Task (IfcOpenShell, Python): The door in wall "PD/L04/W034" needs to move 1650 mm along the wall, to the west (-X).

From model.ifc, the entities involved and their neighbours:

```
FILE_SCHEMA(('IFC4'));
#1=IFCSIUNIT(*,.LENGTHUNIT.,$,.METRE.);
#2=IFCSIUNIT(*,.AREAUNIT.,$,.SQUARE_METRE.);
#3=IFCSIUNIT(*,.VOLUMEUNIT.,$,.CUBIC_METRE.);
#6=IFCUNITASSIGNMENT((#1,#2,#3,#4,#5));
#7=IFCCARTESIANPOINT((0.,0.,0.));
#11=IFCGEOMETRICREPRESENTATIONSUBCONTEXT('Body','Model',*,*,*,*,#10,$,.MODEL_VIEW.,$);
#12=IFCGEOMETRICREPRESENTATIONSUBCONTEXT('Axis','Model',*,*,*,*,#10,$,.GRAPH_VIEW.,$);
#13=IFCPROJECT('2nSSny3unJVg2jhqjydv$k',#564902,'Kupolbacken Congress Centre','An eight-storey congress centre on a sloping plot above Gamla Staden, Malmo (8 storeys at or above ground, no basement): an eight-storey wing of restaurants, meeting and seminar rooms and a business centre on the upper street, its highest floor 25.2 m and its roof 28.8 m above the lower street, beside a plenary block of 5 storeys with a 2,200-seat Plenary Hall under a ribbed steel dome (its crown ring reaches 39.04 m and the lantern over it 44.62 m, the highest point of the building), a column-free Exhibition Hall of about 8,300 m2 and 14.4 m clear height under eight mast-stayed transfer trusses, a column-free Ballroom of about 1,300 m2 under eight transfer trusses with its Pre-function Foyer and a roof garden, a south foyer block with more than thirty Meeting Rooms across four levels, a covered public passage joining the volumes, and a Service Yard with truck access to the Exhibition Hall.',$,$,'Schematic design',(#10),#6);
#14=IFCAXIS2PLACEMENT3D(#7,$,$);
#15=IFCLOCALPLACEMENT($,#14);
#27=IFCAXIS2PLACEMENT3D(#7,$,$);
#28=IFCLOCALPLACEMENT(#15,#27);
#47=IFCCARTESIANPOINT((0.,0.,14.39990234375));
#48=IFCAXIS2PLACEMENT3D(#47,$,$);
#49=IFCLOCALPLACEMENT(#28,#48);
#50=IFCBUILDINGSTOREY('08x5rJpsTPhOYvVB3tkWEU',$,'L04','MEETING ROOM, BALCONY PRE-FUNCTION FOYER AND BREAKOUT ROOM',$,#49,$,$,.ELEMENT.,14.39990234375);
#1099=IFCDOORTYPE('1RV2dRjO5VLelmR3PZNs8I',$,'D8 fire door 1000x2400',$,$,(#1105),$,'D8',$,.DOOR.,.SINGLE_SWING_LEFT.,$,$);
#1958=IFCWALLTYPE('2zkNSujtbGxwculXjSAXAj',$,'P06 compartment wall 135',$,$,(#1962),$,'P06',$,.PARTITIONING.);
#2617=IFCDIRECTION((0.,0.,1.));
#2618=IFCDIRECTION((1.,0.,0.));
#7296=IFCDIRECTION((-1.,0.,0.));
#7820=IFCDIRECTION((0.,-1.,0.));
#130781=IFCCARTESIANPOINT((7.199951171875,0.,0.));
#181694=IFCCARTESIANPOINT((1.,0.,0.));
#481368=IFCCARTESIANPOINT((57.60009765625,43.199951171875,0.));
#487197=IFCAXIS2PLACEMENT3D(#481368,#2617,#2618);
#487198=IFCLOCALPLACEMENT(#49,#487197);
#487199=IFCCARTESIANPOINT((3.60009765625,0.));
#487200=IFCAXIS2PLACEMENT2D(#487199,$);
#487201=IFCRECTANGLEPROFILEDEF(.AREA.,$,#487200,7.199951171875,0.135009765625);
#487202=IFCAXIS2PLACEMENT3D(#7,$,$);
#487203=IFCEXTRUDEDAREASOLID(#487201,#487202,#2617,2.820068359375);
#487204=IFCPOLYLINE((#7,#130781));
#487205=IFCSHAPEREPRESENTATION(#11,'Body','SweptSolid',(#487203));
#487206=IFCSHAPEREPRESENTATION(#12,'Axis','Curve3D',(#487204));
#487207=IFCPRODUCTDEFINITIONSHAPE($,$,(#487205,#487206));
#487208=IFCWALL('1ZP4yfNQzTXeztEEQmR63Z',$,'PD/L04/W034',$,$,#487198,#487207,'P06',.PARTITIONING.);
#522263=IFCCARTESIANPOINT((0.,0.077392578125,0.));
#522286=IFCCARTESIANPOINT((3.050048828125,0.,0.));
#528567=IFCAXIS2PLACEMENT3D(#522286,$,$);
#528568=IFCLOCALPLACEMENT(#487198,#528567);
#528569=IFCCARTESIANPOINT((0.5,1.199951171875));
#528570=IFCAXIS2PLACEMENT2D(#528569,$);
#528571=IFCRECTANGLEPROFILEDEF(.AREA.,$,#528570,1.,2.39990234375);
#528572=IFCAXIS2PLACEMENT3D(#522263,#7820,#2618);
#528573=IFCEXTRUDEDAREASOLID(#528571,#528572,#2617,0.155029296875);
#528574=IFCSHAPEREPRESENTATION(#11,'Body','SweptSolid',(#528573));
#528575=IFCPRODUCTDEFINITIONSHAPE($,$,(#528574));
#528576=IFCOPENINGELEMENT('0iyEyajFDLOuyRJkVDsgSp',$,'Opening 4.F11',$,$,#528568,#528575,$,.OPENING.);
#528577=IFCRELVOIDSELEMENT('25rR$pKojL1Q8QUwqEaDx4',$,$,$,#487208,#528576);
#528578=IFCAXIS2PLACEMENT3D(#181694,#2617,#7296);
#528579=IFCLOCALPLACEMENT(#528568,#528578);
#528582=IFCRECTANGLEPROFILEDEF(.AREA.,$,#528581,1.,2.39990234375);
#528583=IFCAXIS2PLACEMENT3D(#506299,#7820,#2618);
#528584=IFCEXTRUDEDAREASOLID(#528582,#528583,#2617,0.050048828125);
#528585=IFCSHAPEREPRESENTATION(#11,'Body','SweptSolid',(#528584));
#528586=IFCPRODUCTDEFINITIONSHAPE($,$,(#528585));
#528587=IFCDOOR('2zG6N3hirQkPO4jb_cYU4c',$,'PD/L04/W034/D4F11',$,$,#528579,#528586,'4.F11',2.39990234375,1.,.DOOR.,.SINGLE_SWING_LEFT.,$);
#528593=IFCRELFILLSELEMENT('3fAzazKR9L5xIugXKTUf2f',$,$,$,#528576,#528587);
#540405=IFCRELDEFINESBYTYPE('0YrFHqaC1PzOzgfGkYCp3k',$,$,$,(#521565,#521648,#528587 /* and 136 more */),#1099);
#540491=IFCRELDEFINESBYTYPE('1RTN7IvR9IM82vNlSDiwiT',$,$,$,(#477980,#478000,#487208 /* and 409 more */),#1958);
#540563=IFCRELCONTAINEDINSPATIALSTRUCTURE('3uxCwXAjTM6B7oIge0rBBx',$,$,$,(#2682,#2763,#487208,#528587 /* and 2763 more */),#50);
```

```python
import ifcopenshell
import ifcopenshell.api.geometry
import ifcopenshell.util.placement
import ifcopenshell.util.unit

model = ifcopenshell.open("model.ifc")
unit_scale = ifcopenshell.util.unit.calculate_unit_scale(model)

door = model.by_guid("2zG6N3hirQkPO4jb_cYU4c")
opening = door.FillsVoids[0].RelatingOpeningElement
wall = opening.VoidsElements[0].RelatingBuildingElement

wall_matrix = ifcopenshell.util.placement.get_local_placement(wall.ObjectPlacement)
shift = wall_matrix[:3, 0] * -1.65 / unit_scale
before = ifcopenshell.util.placement.get_local_placement(door.ObjectPlacement)[:3, 3].copy()

# The door is placed relative to its opening, so it follows when the opening moves.
matrix = ifcopenshell.util.placement.get_local_placement(opening.ObjectPlacement)
matrix[:3, 3] += shift
ifcopenshell.api.geometry.edit_object_placement(
    model, product=opening, matrix=matrix, is_si=False, should_transform_children=True
)

after = ifcopenshell.util.placement.get_local_placement(door.ObjectPlacement)[:3, 3]
print("door moved by", (after - before).round(3) + 0.0)

model.write("model_edited.ifc")
```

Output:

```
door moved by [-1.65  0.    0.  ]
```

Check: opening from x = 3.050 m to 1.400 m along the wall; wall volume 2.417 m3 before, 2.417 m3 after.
